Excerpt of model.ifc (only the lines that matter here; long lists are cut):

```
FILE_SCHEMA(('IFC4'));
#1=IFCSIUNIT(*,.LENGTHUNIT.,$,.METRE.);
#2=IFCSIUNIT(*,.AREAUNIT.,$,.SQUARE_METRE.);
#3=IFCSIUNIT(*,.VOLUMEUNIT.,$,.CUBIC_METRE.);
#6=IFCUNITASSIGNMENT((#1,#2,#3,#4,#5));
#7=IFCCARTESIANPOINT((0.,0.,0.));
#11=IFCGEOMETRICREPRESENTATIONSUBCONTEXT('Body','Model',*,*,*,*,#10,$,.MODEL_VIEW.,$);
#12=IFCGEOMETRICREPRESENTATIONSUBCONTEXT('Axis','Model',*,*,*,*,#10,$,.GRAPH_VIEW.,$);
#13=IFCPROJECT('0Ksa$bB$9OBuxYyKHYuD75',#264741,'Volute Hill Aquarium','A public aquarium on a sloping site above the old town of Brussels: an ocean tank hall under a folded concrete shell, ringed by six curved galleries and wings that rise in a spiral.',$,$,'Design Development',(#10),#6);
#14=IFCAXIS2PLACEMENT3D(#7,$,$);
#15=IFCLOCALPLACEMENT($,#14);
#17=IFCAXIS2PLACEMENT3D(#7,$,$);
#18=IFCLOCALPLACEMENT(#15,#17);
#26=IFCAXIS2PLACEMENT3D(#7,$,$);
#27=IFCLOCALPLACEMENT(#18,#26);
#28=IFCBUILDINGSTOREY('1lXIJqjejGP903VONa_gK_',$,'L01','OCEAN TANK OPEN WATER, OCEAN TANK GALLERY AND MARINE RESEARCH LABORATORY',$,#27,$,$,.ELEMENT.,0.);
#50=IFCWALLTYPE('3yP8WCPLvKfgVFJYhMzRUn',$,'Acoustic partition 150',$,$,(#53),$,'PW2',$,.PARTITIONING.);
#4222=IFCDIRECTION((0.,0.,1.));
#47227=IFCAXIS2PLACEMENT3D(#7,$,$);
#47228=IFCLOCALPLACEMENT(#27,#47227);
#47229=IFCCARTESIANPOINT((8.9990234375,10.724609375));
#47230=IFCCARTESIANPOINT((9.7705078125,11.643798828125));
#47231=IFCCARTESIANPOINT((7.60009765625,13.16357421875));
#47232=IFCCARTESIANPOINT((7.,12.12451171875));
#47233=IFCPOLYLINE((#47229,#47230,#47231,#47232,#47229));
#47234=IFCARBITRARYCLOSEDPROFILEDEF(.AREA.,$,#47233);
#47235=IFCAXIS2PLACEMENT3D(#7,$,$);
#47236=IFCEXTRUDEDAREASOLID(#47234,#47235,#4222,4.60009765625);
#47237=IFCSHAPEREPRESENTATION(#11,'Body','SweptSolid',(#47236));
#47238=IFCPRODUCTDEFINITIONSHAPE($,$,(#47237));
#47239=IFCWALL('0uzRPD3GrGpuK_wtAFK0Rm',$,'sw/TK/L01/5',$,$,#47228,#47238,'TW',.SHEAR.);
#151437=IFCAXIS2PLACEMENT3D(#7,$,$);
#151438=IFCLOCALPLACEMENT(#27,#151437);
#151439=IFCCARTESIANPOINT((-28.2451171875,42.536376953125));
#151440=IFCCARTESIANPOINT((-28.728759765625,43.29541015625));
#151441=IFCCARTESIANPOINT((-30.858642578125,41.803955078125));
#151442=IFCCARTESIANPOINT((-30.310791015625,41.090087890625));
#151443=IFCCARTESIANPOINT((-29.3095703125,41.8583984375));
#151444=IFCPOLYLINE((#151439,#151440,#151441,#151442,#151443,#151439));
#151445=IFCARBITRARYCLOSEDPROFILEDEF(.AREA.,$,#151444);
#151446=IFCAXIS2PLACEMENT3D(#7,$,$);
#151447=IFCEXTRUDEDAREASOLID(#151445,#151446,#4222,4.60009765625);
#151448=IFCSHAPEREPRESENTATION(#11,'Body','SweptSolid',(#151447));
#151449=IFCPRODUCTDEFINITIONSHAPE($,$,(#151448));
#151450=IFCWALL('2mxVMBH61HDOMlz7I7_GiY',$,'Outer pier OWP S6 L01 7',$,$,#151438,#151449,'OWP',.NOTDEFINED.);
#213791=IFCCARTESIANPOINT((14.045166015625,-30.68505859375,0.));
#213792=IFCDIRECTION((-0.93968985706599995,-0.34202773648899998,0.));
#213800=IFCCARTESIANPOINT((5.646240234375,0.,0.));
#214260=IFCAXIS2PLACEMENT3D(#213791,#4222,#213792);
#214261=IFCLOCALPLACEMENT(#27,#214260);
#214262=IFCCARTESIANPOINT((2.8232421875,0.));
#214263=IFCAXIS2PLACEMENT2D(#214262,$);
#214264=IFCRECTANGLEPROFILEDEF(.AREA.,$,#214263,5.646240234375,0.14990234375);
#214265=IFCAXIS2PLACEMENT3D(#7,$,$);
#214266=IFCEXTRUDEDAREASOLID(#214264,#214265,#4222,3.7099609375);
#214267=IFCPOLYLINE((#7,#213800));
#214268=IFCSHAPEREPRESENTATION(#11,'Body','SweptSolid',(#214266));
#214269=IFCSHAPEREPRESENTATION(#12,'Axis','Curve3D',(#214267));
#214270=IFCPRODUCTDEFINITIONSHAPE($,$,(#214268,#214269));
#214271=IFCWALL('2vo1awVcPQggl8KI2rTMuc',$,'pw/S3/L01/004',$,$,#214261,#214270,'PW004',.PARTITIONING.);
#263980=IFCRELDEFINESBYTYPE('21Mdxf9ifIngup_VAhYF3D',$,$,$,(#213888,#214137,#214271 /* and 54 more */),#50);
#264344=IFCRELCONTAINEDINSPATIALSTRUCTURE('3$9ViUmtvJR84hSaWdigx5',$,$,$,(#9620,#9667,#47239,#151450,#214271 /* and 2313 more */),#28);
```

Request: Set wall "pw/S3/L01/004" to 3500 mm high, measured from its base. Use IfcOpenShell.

```python
import ifcopenshell
import ifcopenshell.geom
import ifcopenshell.util.representation
import ifcopenshell.util.shape

model = ifcopenshell.open("model.ifc")
settings = ifcopenshell.geom.settings()


def volume(element):
    """Net volume in cubic metres, openings subtracted."""
    shape = ifcopenshell.geom.create_shape(settings, element)
    return ifcopenshell.util.shape.get_volume(shape.geometry)


wall = model.by_id(214271)
before = volume(wall)

body = ifcopenshell.util.representation.get_representation(wall, "Model", "Body")
solid = body.Items[0]
old_height = solid.Depth
solid.Depth = 3.5
after = volume(wall)

print(f"height {old_height:g} -> {solid.Depth:g}, volume {before:.3f} -> {after:.3f} m3")

model.write("model_edited.ifc")
```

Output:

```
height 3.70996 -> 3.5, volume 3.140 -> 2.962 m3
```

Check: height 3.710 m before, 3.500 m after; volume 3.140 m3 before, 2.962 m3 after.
